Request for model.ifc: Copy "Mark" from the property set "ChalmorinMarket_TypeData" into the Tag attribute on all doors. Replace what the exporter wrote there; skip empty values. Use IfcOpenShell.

First a look at what the model holds.

```python
import ifcopenshell
import ifcopenshell.util.element

model = ifcopenshell.open("model.ifc")
print(model.schema)
doors = model.by_type("IfcDoor")
print(len(doors), "doors")
for e in doors[:8]:
    source = ifcopenshell.util.element.get_pset(e, "ChalmorinMarket_TypeData", "Mark")
    target = e.Tag
    print(e.id(), repr(source), repr(target), sep=" | ")
```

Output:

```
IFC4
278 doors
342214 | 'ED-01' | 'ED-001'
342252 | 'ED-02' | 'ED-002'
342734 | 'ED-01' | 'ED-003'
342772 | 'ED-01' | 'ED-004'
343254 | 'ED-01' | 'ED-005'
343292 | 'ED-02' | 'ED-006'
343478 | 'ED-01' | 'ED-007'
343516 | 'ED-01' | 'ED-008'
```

```python
import ifcopenshell
import ifcopenshell.util.element

model = ifcopenshell.open("model.ifc")

count = 0
for e in model.by_type("IfcDoor"):
    value = ifcopenshell.util.element.get_pset(e, "ChalmorinMarket_TypeData", "Mark")
    current = e.Tag
    if not value or not value.strip() or current == value:
        continue
    e.Tag = value
    count += 1

print(count, "doors updated")

model.write("model_updated.ifc")
```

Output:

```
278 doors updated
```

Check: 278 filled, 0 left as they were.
